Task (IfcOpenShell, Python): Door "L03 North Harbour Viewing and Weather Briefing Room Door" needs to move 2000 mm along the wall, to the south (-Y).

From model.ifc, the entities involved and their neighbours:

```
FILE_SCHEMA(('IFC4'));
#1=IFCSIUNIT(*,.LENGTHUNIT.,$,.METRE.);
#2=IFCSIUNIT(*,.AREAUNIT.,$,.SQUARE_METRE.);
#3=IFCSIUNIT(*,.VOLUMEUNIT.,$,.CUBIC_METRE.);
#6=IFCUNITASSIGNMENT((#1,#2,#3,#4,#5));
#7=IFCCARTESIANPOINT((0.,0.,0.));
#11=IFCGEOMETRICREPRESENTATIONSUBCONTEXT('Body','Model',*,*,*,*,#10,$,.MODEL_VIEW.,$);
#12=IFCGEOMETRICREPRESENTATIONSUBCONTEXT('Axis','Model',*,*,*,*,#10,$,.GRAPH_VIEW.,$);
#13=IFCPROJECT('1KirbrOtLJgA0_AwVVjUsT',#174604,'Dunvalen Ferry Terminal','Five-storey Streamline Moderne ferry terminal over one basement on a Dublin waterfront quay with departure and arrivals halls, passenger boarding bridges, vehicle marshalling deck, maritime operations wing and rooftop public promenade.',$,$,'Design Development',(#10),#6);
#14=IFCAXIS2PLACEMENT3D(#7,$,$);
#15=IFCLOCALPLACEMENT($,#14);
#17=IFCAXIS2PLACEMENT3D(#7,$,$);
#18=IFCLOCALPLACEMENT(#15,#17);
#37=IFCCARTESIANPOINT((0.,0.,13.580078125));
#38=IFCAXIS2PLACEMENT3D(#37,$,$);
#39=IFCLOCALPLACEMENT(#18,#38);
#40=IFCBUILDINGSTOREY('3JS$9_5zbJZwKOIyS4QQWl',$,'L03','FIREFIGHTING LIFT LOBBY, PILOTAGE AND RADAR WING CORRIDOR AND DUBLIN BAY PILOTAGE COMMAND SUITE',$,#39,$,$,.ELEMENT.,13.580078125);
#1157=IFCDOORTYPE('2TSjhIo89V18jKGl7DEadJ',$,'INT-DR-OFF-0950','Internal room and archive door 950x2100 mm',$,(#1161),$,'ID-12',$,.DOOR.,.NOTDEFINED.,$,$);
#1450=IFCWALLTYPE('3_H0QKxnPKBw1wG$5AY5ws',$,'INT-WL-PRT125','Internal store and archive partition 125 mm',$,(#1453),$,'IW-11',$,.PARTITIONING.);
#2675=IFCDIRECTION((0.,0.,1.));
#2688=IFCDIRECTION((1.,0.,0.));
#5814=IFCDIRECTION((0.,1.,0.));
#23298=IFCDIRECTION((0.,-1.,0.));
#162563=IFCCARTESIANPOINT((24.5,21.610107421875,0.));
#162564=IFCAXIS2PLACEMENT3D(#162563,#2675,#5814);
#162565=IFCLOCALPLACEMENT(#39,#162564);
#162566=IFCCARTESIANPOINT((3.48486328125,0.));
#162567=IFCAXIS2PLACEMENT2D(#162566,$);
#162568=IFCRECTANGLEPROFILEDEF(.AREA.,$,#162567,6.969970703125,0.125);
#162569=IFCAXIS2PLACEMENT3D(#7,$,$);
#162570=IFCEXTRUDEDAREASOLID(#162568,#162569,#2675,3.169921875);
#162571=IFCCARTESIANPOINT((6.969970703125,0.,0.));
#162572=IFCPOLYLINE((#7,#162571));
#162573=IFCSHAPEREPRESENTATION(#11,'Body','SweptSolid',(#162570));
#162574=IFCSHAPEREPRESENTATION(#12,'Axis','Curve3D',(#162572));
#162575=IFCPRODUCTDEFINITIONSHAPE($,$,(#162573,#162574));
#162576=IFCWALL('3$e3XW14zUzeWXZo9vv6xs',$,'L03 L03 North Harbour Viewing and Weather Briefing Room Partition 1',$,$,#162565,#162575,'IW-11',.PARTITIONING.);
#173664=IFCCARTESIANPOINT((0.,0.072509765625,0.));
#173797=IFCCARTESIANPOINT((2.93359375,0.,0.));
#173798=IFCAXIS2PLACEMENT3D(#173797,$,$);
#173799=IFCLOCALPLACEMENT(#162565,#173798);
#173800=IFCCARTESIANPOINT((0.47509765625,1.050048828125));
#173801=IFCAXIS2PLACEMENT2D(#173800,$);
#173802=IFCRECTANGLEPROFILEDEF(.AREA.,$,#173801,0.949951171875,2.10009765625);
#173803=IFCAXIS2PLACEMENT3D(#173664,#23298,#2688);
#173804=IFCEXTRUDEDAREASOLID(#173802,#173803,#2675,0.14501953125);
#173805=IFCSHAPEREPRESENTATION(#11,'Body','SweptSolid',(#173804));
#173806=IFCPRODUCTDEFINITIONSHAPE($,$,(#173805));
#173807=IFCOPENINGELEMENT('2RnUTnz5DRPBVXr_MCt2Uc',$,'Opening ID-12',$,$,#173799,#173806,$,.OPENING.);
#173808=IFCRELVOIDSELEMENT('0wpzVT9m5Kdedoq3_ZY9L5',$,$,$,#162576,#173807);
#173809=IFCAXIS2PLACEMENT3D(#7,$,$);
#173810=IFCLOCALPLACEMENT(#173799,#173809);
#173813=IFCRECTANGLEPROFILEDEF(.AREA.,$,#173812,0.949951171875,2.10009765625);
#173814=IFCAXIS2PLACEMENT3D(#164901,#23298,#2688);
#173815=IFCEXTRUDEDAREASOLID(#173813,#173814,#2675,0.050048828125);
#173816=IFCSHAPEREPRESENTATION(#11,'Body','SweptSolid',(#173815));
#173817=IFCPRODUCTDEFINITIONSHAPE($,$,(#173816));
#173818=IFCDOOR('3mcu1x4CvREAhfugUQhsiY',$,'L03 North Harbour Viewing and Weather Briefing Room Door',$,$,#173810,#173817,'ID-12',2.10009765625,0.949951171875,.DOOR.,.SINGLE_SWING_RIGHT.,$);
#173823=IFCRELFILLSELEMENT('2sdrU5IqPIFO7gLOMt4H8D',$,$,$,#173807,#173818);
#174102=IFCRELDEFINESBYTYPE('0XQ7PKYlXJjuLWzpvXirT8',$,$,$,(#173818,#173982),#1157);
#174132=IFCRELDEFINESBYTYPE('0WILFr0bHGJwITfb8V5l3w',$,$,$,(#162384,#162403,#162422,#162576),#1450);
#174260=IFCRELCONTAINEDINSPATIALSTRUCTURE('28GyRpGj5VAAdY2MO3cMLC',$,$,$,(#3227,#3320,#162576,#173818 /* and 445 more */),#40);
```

```python
import ifcopenshell
import ifcopenshell.api.geometry
import ifcopenshell.util.placement
import ifcopenshell.util.unit

model = ifcopenshell.open("model.ifc")
unit_scale = ifcopenshell.util.unit.calculate_unit_scale(model)

door = model.by_guid("3mcu1x4CvREAhfugUQhsiY")
opening = door.FillsVoids[0].RelatingOpeningElement
wall = opening.VoidsElements[0].RelatingBuildingElement

wall_matrix = ifcopenshell.util.placement.get_local_placement(wall.ObjectPlacement)
shift = wall_matrix[:3, 0] * -2 / unit_scale
before = ifcopenshell.util.placement.get_local_placement(door.ObjectPlacement)[:3, 3].copy()

# The door is placed relative to its opening, so it follows when the opening moves.
matrix = ifcopenshell.util.placement.get_local_placement(opening.ObjectPlacement)
matrix[:3, 3] += shift
ifcopenshell.api.geometry.edit_object_placement(
    model, product=opening, matrix=matrix, is_si=False, should_transform_children=True
)

after = ifcopenshell.util.placement.get_local_placement(door.ObjectPlacement)[:3, 3]
print("door moved by", (after - before).round(3) + 0.0)

model.write("model_rev.ifc")
```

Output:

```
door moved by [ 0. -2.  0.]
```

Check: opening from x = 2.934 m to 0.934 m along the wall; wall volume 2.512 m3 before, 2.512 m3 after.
